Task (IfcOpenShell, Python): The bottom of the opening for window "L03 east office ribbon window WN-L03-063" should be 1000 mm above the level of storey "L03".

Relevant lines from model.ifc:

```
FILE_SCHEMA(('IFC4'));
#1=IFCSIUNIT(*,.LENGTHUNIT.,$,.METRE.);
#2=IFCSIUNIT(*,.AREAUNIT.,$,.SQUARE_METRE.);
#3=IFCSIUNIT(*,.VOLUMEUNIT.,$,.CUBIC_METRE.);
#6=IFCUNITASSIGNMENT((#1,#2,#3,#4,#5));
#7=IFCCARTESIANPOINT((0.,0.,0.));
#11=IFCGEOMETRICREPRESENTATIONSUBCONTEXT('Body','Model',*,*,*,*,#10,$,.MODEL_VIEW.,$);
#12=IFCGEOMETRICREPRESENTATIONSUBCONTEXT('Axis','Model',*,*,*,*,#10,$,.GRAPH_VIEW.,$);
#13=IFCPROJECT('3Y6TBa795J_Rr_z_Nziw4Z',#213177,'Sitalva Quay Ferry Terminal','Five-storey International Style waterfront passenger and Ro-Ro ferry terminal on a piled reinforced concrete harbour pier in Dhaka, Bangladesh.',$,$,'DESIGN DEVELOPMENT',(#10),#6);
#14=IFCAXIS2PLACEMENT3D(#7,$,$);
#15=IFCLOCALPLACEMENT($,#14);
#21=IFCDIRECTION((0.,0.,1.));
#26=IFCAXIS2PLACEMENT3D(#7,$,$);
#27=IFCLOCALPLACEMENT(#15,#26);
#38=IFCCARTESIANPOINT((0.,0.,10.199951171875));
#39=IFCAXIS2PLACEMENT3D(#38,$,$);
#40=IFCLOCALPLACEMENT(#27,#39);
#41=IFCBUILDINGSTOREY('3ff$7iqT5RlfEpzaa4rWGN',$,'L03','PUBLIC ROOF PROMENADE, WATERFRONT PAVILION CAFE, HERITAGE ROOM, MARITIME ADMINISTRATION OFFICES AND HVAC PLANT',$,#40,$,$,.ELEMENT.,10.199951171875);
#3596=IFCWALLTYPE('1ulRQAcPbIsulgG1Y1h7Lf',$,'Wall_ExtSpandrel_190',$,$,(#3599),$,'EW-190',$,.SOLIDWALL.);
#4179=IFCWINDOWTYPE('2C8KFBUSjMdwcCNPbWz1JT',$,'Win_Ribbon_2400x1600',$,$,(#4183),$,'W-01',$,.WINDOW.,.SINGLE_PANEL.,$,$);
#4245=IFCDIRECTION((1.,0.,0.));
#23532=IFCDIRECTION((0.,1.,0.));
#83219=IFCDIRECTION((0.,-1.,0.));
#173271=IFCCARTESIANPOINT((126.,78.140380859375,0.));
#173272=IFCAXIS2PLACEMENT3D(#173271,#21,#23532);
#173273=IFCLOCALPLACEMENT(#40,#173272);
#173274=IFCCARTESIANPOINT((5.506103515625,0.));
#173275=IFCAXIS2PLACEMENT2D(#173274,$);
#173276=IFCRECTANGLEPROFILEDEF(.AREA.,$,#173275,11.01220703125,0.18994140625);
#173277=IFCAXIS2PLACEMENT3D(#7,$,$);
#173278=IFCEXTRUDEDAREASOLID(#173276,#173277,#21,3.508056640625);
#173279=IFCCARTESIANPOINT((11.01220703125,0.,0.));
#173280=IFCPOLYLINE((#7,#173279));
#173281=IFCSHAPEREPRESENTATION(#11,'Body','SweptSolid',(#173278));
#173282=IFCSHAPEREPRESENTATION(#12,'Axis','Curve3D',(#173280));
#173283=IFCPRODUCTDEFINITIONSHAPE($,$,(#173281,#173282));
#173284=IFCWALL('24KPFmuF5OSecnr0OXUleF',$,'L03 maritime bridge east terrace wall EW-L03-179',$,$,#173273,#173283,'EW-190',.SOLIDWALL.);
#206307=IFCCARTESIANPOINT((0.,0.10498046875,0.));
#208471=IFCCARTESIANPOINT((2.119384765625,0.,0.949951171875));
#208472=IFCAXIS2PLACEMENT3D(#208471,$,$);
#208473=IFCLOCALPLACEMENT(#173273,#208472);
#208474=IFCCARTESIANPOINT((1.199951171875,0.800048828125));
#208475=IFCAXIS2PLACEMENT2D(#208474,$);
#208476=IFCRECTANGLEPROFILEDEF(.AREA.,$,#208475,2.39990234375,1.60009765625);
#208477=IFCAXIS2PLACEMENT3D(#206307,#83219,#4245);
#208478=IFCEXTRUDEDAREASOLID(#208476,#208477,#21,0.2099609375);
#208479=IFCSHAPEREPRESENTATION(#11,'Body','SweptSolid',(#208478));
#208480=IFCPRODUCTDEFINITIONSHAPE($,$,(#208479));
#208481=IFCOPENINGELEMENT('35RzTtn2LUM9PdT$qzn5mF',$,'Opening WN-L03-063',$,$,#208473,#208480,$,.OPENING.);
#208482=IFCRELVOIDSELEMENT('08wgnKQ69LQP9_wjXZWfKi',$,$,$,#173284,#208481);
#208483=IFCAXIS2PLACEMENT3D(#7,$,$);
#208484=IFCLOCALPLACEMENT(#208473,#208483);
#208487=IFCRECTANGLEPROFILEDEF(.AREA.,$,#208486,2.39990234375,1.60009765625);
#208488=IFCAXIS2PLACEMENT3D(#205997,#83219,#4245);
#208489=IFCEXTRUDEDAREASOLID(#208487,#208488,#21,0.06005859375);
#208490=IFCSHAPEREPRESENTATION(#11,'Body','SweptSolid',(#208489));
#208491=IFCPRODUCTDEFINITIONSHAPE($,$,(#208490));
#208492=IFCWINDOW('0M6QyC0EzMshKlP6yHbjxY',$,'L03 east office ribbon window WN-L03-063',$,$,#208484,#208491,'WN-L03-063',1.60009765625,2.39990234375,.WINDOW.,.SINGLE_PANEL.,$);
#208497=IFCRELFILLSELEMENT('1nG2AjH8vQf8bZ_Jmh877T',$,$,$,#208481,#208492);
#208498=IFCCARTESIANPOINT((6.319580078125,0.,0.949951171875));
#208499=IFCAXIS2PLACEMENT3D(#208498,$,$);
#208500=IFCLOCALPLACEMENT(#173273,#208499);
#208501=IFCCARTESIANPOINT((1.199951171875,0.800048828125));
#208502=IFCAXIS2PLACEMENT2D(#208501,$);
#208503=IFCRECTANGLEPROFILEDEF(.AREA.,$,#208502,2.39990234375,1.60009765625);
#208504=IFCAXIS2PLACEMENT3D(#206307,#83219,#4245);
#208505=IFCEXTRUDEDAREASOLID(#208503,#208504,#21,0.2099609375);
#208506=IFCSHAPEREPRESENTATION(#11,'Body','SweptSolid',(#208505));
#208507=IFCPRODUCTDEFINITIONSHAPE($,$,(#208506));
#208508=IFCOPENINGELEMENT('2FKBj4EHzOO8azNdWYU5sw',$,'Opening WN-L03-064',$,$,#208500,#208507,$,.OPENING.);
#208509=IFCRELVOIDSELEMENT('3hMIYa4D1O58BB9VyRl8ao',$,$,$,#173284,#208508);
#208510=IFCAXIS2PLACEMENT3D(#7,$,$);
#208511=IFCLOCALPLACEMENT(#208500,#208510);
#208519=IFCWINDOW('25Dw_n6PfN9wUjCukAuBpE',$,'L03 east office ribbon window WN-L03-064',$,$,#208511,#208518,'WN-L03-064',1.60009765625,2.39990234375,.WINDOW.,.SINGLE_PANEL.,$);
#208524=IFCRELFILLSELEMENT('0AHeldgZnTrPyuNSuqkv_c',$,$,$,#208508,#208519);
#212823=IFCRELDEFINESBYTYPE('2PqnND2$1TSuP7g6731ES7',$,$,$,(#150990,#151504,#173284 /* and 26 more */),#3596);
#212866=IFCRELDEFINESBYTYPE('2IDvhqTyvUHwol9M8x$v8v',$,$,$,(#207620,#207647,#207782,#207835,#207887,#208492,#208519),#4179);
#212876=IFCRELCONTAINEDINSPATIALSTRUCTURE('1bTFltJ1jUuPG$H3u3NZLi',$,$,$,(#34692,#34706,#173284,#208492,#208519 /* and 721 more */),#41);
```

```python
import numpy as np
import ifcopenshell
import ifcopenshell.api.geometry
import ifcopenshell.geom
import ifcopenshell.util.element
import ifcopenshell.util.placement
import ifcopenshell.util.shape
import ifcopenshell.util.unit

model = ifcopenshell.open("model.ifc")
unit_scale = ifcopenshell.util.unit.calculate_unit_scale(model)

window = model.by_guid("0M6QyC0EzMshKlP6yHbjxY")
opening = window.FillsVoids[0].RelatingOpeningElement
storey = ifcopenshell.util.element.get_container(window, ifc_class="IfcBuildingStorey")
level = ifcopenshell.util.placement.get_local_placement(storey.ObjectPlacement)[2, 3]

# The opening's origin need not be at the sill, so measure its lowest point.
shape = ifcopenshell.geom.create_shape(ifcopenshell.geom.settings(), opening)
bottom = ifcopenshell.util.shape.get_shape_bottom_elevation(shape, shape.geometry) / unit_scale
dz = level + 1 / unit_scale - bottom

shift = np.array([0.0, 0.0, dz])
# The window is placed relative to its opening, so it follows when the opening moves.
matrix = ifcopenshell.util.placement.get_local_placement(opening.ObjectPlacement)
matrix[:3, 3] += shift
ifcopenshell.api.geometry.edit_object_placement(
    model, product=opening, matrix=matrix, is_si=False, should_transform_children=True
)

print(f"moved by {dz * unit_scale:+.3f} m")

model.write("model-out.ifc")
```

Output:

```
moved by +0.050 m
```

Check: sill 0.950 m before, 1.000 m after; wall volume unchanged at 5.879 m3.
